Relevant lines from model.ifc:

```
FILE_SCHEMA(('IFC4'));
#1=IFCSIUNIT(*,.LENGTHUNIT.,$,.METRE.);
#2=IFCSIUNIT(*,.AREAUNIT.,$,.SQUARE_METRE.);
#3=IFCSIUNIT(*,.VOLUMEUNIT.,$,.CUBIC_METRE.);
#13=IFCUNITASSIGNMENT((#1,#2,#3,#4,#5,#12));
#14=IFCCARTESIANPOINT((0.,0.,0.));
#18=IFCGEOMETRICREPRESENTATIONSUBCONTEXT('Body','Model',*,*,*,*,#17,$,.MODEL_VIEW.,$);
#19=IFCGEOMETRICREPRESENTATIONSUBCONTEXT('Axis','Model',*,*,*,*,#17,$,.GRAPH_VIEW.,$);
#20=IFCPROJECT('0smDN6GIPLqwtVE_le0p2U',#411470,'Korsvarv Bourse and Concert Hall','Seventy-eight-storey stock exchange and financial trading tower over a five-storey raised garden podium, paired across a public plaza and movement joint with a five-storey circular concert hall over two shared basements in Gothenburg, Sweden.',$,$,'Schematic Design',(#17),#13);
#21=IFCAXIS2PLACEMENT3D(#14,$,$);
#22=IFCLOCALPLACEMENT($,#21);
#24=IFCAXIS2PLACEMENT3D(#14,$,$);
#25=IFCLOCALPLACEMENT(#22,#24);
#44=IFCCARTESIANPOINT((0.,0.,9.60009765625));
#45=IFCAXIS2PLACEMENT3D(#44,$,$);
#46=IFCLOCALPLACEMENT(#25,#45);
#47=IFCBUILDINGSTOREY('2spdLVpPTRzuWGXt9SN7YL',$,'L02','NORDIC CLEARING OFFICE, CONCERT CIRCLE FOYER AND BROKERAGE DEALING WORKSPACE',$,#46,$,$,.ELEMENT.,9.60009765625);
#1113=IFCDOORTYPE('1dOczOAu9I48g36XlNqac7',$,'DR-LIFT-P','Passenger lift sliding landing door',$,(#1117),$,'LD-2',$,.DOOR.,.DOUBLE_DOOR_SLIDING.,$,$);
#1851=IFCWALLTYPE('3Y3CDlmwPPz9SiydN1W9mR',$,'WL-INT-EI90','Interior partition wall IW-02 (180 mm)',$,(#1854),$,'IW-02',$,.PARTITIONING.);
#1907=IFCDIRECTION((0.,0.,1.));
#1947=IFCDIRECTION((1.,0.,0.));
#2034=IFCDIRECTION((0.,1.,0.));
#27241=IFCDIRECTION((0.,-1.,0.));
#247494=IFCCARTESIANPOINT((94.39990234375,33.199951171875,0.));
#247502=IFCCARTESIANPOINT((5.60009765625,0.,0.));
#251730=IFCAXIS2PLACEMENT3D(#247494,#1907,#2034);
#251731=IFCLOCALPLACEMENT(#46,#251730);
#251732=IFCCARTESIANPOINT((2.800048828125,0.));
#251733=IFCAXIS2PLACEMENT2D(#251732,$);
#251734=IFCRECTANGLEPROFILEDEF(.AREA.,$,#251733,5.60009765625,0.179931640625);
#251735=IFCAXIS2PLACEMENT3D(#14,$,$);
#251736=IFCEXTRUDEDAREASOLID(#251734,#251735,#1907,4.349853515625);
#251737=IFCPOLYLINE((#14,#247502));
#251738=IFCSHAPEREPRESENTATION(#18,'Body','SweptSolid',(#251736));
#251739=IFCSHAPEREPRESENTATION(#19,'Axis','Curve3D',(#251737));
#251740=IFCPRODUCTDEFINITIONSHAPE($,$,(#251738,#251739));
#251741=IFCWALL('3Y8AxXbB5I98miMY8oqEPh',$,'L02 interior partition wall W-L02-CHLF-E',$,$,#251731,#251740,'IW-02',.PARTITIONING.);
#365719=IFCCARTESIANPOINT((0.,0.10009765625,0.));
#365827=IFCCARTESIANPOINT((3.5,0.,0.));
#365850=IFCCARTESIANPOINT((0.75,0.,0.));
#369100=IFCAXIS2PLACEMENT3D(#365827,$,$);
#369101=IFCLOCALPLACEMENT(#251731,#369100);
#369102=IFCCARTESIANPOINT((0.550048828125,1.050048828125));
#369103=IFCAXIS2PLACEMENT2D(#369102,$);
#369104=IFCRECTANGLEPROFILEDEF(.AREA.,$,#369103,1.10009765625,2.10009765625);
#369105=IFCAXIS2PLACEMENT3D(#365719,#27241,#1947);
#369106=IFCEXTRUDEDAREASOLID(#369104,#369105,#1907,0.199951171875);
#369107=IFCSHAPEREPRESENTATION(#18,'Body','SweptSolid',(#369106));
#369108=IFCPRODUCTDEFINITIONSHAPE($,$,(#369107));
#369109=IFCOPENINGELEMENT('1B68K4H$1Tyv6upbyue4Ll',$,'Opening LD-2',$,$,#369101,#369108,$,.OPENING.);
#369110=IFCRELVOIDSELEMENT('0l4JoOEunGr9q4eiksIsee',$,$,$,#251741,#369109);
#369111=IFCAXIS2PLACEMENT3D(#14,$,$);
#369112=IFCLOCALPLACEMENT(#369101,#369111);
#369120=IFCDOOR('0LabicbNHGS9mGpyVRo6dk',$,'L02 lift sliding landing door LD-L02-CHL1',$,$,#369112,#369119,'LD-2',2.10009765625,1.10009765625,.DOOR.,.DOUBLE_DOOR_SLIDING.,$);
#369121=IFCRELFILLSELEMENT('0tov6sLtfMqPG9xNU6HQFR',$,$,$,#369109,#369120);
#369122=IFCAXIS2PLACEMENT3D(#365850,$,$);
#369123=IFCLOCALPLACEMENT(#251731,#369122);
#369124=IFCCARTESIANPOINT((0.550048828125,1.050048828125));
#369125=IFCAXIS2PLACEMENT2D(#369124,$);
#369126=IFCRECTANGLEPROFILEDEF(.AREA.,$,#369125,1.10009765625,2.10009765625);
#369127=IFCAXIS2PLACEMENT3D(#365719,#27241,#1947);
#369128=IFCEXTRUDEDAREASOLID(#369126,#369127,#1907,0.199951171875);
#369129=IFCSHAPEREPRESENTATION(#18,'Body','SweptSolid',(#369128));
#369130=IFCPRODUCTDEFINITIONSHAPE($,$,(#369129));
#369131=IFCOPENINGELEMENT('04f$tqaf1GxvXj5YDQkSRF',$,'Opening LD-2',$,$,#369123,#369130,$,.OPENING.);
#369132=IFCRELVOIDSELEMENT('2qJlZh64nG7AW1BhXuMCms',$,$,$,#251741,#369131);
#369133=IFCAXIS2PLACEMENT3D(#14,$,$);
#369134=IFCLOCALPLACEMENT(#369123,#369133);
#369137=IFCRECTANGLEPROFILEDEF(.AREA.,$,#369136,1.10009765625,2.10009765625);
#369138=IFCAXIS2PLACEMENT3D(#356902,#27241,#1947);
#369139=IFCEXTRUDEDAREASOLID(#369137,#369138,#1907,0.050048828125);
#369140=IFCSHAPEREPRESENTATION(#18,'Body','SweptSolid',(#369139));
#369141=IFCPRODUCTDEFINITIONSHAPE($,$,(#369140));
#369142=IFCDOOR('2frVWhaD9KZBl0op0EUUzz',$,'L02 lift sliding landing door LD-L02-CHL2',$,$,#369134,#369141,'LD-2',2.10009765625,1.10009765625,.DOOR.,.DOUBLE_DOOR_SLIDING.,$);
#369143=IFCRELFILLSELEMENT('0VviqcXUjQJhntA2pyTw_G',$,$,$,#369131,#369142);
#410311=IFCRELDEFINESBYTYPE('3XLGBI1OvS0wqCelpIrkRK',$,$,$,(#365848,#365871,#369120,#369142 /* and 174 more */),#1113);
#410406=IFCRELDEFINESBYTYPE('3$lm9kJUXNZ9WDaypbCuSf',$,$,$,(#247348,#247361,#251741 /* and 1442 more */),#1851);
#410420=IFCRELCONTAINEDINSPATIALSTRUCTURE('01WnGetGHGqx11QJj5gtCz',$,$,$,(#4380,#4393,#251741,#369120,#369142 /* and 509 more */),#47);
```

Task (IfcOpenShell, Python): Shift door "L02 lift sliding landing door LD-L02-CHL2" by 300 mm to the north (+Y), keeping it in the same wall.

```python
import ifcopenshell
import ifcopenshell.api.geometry
import ifcopenshell.util.placement
import ifcopenshell.util.unit

model = ifcopenshell.open("model.ifc")
unit_scale = ifcopenshell.util.unit.calculate_unit_scale(model)

door = model.by_guid("2frVWhaD9KZBl0op0EUUzz")
opening = door.FillsVoids[0].RelatingOpeningElement
wall = opening.VoidsElements[0].RelatingBuildingElement

wall_matrix = ifcopenshell.util.placement.get_local_placement(wall.ObjectPlacement)
shift = wall_matrix[:3, 0] * 0.3 / unit_scale
before = ifcopenshell.util.placement.get_local_placement(door.ObjectPlacement)[:3, 3].copy()

# The door is placed relative to its opening, so it follows when the opening moves.
matrix = ifcopenshell.util.placement.get_local_placement(opening.ObjectPlacement)
matrix[:3, 3] += shift
ifcopenshell.api.geometry.edit_object_placement(
    model, product=opening, matrix=matrix, is_si=False, should_transform_children=True
)

after = ifcopenshell.util.placement.get_local_placement(door.ObjectPlacement)[:3, 3]
print("door moved by", (after - before).round(3) + 0.0)

model.write("model_rev.ifc")
```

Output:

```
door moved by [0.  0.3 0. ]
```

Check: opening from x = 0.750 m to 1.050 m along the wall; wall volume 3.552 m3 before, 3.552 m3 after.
